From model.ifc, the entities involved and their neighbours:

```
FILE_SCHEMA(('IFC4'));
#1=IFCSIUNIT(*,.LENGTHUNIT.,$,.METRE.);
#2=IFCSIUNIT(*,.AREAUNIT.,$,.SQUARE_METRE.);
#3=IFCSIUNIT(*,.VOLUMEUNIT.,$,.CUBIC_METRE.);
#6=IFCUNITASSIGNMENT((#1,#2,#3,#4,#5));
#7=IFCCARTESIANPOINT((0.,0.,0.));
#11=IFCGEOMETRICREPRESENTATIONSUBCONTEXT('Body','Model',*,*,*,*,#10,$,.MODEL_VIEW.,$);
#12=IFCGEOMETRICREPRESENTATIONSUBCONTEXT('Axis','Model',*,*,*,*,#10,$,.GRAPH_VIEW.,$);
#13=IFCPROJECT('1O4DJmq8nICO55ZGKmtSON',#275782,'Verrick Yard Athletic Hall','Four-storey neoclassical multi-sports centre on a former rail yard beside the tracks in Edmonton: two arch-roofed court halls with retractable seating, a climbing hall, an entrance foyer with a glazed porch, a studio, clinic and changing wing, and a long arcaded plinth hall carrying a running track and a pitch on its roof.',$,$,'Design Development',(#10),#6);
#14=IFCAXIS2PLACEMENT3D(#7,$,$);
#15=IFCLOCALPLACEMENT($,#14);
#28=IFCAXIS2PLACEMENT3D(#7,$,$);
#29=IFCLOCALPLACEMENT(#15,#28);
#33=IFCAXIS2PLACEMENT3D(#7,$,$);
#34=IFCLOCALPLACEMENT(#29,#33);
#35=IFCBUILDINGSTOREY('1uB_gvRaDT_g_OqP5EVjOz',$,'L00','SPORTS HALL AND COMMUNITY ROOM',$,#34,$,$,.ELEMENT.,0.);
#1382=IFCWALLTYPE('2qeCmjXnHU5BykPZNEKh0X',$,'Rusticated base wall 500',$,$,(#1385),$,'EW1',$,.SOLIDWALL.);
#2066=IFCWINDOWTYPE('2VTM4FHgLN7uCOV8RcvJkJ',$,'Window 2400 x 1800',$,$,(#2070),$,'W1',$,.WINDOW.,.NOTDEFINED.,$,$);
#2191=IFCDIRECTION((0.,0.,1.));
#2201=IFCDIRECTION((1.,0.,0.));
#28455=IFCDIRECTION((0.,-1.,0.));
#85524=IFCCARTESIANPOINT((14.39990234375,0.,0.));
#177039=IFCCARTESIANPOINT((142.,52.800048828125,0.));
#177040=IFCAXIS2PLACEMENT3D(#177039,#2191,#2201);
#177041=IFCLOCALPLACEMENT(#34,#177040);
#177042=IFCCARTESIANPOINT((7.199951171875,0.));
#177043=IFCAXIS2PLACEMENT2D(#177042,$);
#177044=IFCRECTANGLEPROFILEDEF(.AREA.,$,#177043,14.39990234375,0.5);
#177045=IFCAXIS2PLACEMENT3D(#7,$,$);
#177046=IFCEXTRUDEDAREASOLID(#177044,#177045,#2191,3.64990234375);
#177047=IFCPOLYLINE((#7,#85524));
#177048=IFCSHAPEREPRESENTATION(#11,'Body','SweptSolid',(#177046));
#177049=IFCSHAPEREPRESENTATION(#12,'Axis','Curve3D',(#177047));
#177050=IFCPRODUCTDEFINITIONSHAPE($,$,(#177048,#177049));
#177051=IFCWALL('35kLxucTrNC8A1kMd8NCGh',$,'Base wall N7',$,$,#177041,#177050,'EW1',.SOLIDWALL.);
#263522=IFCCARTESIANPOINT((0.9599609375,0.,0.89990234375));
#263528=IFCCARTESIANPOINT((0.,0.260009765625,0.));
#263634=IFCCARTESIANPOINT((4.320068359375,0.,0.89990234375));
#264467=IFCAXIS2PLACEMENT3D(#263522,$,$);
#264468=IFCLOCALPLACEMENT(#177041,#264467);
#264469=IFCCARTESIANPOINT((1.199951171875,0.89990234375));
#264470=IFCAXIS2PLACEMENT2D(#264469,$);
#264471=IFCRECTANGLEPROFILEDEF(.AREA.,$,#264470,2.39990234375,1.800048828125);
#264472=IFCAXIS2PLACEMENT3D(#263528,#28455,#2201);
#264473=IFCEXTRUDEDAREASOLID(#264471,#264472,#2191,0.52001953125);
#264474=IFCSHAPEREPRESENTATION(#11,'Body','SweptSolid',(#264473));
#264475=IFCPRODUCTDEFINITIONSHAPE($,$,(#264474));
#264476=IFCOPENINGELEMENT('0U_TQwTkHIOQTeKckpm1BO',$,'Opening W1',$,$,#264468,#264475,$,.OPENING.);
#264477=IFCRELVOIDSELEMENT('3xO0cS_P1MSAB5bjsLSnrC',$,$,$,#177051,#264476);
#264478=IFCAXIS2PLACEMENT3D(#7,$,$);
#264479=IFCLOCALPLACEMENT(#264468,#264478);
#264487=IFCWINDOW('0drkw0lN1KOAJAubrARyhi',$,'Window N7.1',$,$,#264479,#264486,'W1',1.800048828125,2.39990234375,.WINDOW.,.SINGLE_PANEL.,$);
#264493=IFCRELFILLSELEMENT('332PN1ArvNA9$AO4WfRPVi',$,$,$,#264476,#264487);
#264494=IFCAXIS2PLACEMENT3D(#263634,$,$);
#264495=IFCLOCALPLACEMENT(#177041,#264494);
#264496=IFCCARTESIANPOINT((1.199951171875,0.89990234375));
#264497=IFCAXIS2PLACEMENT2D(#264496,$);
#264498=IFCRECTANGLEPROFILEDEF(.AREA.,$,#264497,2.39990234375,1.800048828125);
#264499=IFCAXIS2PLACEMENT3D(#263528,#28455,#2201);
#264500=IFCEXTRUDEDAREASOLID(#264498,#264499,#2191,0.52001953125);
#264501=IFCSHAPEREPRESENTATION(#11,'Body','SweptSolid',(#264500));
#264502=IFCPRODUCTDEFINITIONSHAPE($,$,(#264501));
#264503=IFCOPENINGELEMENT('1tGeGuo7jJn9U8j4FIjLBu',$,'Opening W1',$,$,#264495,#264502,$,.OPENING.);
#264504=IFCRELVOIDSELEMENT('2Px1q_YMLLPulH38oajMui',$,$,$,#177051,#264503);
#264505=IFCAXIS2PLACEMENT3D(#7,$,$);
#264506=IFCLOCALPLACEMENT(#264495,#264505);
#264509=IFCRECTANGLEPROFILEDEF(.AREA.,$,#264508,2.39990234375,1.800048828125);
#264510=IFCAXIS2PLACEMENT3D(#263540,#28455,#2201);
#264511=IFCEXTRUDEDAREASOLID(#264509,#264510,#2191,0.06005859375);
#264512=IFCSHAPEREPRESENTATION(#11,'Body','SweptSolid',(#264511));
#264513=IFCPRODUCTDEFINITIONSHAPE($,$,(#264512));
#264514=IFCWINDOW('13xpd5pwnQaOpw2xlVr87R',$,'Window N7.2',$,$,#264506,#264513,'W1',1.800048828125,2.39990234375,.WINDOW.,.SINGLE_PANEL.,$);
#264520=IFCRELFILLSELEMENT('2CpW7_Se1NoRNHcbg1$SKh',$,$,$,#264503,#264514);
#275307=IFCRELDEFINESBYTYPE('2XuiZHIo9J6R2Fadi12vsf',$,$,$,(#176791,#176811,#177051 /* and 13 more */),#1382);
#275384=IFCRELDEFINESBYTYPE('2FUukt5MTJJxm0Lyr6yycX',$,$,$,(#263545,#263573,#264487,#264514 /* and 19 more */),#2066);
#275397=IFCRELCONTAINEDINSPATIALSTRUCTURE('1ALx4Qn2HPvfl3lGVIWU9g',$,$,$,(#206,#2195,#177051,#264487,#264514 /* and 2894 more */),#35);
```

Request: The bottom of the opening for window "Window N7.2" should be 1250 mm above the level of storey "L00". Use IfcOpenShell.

```python
import numpy as np
import ifcopenshell
import ifcopenshell.api.geometry
import ifcopenshell.geom
import ifcopenshell.util.element
import ifcopenshell.util.placement
import ifcopenshell.util.shape
import ifcopenshell.util.unit

model = ifcopenshell.open("model.ifc")
unit_scale = ifcopenshell.util.unit.calculate_unit_scale(model)

window = model.by_guid("13xpd5pwnQaOpw2xlVr87R")
opening = window.FillsVoids[0].RelatingOpeningElement
storey = ifcopenshell.util.element.get_container(window, ifc_class="IfcBuildingStorey")
level = ifcopenshell.util.placement.get_local_placement(storey.ObjectPlacement)[2, 3]

# The opening's origin need not be at the sill, so measure its lowest point.
shape = ifcopenshell.geom.create_shape(ifcopenshell.geom.settings(), opening)
bottom = ifcopenshell.util.shape.get_shape_bottom_elevation(shape, shape.geometry) / unit_scale
dz = level + 1.25 - bottom

shift = np.array([0.0, 0.0, dz])
# The window is placed relative to its opening, so it follows when the opening moves.
matrix = ifcopenshell.util.placement.get_local_placement(opening.ObjectPlacement)
matrix[:3, 3] += shift
ifcopenshell.api.geometry.edit_object_placement(
    model, product=opening, matrix=matrix, is_si=False, should_transform_children=True
)

print(f"moved by {dz * unit_scale:+.3f} m")

model.write("model_edited.ifc")
```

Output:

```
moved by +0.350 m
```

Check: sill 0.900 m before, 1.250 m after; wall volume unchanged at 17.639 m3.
